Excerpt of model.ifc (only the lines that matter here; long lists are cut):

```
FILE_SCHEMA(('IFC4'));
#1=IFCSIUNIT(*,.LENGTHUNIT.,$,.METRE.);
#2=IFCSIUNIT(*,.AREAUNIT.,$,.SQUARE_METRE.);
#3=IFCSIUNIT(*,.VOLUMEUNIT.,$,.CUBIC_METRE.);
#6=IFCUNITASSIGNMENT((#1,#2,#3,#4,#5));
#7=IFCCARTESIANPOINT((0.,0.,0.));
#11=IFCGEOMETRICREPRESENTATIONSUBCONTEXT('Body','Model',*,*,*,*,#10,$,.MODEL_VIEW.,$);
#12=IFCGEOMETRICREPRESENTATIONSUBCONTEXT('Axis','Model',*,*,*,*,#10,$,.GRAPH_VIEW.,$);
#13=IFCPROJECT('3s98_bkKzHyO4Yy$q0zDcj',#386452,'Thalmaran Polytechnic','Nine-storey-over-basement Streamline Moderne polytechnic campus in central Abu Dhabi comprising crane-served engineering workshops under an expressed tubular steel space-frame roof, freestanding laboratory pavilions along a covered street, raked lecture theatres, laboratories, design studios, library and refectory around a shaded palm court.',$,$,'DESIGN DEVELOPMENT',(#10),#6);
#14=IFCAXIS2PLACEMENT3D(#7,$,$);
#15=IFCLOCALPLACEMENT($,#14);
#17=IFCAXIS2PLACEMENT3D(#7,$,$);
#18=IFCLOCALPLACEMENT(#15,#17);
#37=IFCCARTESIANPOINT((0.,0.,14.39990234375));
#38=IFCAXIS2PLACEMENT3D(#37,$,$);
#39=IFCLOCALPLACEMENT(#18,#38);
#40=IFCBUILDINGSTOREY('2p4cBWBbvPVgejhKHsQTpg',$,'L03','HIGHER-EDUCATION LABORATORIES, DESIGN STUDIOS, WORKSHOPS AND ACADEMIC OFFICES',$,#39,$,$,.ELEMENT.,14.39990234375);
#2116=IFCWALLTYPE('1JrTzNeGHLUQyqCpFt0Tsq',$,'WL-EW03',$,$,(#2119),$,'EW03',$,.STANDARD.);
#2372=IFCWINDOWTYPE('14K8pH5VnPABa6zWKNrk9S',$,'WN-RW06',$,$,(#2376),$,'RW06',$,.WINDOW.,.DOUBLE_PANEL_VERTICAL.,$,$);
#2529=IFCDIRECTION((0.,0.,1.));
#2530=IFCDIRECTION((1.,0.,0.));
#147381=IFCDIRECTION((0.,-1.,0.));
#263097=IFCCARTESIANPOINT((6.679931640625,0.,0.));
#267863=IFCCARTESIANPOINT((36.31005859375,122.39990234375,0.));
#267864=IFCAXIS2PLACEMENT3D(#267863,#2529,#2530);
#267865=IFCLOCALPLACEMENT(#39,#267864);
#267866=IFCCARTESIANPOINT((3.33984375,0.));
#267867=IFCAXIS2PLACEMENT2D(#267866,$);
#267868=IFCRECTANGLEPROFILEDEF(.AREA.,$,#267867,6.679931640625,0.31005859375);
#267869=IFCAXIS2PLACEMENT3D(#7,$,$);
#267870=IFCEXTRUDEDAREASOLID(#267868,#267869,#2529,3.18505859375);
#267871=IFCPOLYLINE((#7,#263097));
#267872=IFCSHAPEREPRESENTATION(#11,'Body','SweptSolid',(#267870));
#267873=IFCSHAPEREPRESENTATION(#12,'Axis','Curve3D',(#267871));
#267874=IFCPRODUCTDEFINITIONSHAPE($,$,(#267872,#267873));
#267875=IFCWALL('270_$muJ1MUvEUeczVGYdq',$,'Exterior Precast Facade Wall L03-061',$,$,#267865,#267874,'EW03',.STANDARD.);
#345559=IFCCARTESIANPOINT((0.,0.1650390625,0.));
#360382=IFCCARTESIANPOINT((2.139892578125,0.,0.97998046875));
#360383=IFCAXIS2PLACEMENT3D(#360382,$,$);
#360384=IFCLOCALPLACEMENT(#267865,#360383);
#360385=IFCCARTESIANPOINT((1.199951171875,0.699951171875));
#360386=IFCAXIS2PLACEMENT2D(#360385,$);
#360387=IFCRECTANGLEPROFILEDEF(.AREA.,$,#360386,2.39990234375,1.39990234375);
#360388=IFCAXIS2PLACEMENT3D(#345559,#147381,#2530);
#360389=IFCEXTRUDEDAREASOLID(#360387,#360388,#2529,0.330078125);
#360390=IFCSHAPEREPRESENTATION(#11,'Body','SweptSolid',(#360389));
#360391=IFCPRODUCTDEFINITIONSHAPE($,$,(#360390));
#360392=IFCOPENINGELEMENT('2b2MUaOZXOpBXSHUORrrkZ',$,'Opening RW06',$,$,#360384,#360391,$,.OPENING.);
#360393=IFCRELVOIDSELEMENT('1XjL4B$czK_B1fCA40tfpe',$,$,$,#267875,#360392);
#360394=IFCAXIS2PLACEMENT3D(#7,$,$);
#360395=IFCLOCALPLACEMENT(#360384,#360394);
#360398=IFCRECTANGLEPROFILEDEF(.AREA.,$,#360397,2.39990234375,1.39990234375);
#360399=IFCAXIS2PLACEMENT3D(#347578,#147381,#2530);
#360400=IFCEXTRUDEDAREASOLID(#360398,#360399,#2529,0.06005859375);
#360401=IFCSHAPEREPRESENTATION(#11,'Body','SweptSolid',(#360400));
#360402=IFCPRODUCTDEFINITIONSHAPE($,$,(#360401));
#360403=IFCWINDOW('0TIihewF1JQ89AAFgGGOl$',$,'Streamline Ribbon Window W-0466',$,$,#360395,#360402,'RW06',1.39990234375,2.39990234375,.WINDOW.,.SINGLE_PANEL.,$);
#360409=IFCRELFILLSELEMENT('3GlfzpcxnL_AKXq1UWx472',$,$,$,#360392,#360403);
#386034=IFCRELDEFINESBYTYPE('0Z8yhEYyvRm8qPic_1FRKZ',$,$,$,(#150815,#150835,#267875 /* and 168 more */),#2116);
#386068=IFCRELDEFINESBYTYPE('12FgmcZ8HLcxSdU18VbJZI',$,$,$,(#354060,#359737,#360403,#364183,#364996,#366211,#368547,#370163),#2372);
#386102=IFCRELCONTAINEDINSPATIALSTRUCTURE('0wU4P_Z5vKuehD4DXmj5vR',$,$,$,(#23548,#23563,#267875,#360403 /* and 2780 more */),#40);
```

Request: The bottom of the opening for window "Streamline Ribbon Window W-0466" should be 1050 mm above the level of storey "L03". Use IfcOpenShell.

```python
import numpy as np
import ifcopenshell
import ifcopenshell.api.geometry
import ifcopenshell.geom
import ifcopenshell.util.element
import ifcopenshell.util.placement
import ifcopenshell.util.shape
import ifcopenshell.util.unit

model = ifcopenshell.open("model.ifc")
unit_scale = ifcopenshell.util.unit.calculate_unit_scale(model)

window = model.by_id(360403)
opening = window.FillsVoids[0].RelatingOpeningElement
storey = ifcopenshell.util.element.get_container(window, ifc_class="IfcBuildingStorey")
level = ifcopenshell.util.placement.get_local_placement(storey.ObjectPlacement)[2, 3]

# The opening's origin need not be at the sill, so measure its lowest point.
shape = ifcopenshell.geom.create_shape(ifcopenshell.geom.settings(), opening)
bottom = ifcopenshell.util.shape.get_shape_bottom_elevation(shape, shape.geometry) / unit_scale
dz = level + 1.05 - bottom

shift = np.array([0.0, 0.0, dz])
# The window is placed relative to its opening, so it follows when the opening moves.
matrix = ifcopenshell.util.placement.get_local_placement(opening.ObjectPlacement)
matrix[:3, 3] += shift
ifcopenshell.api.geometry.edit_object_placement(
    model, product=opening, matrix=matrix, is_si=False, should_transform_children=True
)

print(f"moved by {dz * unit_scale:+.3f} m")

model.write("model_rev.ifc")
```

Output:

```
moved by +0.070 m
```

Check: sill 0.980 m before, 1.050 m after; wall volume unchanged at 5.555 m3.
